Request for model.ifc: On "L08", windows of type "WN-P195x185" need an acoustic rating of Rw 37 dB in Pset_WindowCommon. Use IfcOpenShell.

First a look at what the model holds.

```python
import ifcopenshell
import ifcopenshell.util.element

model = ifcopenshell.open("model.ifc")
print(model.schema)
storey = next(s for s in model.by_type("IfcBuildingStorey") if s.Name == "L08")
windows = [e for e in ifcopenshell.util.element.get_decomposition(storey) if e.is_a("IfcWindow")]
seen = {}
for e in windows:
    element_type = ifcopenshell.util.element.get_type(e)
    key = (element_type.Name if element_type != e and element_type else None, ifcopenshell.util.element.get_pset(e, "Pset_WindowCommon", "AcousticRating"))
    seen[key] = seen.get(key, 0) + 1
for (name, value), count in sorted(seen.items(), key=str):
    print(count, "x", name, "|", value)
```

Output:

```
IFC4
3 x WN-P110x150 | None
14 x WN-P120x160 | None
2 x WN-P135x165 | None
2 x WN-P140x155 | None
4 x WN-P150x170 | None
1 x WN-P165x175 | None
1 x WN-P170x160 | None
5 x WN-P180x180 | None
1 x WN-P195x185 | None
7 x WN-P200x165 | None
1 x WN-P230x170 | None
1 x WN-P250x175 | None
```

```python
import ifcopenshell
import ifcopenshell.api.pset
import ifcopenshell.util.element

model = ifcopenshell.open("model.ifc")

storey = next(s for s in model.by_type("IfcBuildingStorey") if s.Name == "L08")
windows = [e for e in ifcopenshell.util.element.get_decomposition(storey) if e.is_a("IfcWindow")]

count = 0
for e in windows:
    element_type = ifcopenshell.util.element.get_type(e)
    if element_type in (None, e) or element_type.Name != "WN-P195x185":
        continue
    # add_pset returns the element's existing set when there is one.
    pset = ifcopenshell.api.pset.add_pset(model, product=e, name="Pset_WindowCommon")
    ifcopenshell.api.pset.edit_pset(model, pset=pset, properties={"AcousticRating": "Rw 37 dB"})
    count += 1

print(count, "windows updated")

model.write("model_v2.ifc")
```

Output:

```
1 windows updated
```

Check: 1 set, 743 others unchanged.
